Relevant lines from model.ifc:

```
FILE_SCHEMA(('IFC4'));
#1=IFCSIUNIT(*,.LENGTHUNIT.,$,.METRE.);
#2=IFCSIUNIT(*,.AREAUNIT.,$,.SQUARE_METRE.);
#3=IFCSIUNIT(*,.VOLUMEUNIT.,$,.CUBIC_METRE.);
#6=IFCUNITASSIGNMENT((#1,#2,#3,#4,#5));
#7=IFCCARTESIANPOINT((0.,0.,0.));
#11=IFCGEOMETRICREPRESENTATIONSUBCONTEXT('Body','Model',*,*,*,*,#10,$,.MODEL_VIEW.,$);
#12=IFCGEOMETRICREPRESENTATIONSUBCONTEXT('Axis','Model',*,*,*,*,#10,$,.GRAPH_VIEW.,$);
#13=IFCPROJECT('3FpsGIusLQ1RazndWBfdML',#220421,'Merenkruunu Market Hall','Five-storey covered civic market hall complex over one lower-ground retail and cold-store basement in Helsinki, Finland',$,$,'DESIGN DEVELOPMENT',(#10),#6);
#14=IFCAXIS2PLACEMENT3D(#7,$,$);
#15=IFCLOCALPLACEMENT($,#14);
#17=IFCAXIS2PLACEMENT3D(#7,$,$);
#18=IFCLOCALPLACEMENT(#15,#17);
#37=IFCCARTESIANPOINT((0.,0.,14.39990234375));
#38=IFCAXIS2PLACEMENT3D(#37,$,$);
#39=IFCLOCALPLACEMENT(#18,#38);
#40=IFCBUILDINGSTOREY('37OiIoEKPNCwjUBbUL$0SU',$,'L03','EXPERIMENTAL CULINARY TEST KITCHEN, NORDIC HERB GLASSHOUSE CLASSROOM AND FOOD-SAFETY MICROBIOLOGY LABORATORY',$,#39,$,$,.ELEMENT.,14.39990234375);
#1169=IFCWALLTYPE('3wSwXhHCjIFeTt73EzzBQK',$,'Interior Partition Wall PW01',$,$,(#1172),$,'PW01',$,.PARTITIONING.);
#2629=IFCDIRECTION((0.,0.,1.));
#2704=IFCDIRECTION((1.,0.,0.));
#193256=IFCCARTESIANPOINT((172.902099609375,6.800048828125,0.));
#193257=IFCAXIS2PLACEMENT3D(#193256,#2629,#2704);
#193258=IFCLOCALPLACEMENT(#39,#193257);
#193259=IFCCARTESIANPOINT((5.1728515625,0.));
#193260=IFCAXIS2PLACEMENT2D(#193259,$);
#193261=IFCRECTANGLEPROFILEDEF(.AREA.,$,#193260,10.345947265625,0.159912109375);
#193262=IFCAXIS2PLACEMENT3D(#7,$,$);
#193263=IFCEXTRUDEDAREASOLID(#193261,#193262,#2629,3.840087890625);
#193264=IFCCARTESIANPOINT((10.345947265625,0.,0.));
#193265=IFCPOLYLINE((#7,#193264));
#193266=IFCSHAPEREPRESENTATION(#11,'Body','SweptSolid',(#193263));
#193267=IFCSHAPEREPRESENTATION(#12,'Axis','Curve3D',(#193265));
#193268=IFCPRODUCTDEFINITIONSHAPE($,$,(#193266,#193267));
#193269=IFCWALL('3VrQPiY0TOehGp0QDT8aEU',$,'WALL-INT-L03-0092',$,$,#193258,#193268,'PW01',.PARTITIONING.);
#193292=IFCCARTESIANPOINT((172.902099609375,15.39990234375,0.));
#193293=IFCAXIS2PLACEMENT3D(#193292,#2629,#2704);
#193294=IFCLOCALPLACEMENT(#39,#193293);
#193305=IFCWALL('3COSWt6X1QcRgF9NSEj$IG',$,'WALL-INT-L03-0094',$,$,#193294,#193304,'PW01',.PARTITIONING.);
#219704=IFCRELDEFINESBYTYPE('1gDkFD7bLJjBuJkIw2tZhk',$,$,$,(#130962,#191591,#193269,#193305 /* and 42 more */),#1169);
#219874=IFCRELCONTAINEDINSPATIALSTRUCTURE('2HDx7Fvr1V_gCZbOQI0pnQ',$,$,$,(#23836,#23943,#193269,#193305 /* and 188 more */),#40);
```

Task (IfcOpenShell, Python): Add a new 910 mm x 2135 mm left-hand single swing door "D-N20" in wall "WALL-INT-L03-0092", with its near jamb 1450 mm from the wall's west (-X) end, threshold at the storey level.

```python
import numpy as np
import ifcopenshell
import ifcopenshell.api.feature
import ifcopenshell.api.geometry
import ifcopenshell.api.root
import ifcopenshell.api.spatial
import ifcopenshell.geom
import ifcopenshell.util.element
import ifcopenshell.util.placement
import ifcopenshell.util.representation
import ifcopenshell.util.shape
import ifcopenshell.util.unit

model = ifcopenshell.open("model.ifc")
unit_scale = ifcopenshell.util.unit.calculate_unit_scale(model)
settings = ifcopenshell.geom.settings()


def volume(element):
    """Net volume in cubic metres, openings subtracted."""
    shape = ifcopenshell.geom.create_shape(settings, element)
    return ifcopenshell.util.shape.get_volume(shape.geometry)


wall = model.by_id(193269)
storey = ifcopenshell.util.element.get_container(wall, ifc_class="IfcBuildingStorey")
context = ifcopenshell.util.representation.get_context(model, "Model", "Body", "MODEL_VIEW")
before = volume(wall)

width, height, from_end, sill = 0.91, 2.135, 1.45, 0.0  # metres

# The wall runs along its own X axis, and the end named is its -X end.
wall_shape = ifcopenshell.geom.create_shape(settings, wall)
x, y, z = ifcopenshell.util.shape.get_vertices(wall_shape.geometry).T
start = x.min() + from_end
face, thickness = float(y.min()), float(y.max() - y.min())
wall_matrix = ifcopenshell.util.placement.get_local_placement(wall.ObjectPlacement)
level = ifcopenshell.util.placement.get_local_placement(storey.ObjectPlacement)[2, 3]


def in_wall(x, y):
    """Placement at x, y metres in the wall's axes, at sill height."""
    matrix = wall_matrix.copy()
    matrix[:, 3] = wall_matrix @ np.array([x / unit_scale, y / unit_scale, 0.0, 1.0])
    matrix[2, 3] = level + sill / unit_scale
    return matrix


# Opening: a box that overshoots both wall faces by 50 mm.
opening = ifcopenshell.api.root.create_entity(model, ifc_class="IfcOpeningElement", predefined_type="OPENING")
box = ifcopenshell.api.geometry.add_wall_representation(
    model, context=context, length=width, height=height, thickness=thickness + 0.1
)
ifcopenshell.api.geometry.assign_representation(model, product=opening, representation=box)
ifcopenshell.api.geometry.edit_object_placement(model, product=opening, matrix=in_wall(start, face - 0.05), is_si=False)
ifcopenshell.api.feature.add_feature(model, feature=opening, element=wall)

door = ifcopenshell.api.root.create_entity(model, ifc_class="IfcDoor", name="D-N20", predefined_type="DOOR")
door.OverallWidth, door.OverallHeight = width / unit_scale, height / unit_scale
door.OperationType = "SINGLE_SWING_LEFT"
body = ifcopenshell.api.geometry.add_door_representation(
    model,
    context=context,
    overall_width=door.OverallWidth,
    overall_height=door.OverallHeight,
    operation_type="SINGLE_SWING_LEFT",
    lining_properties={"LiningDepth": thickness / unit_scale, "ThresholdDepth": thickness / unit_scale},
)
ifcopenshell.api.geometry.assign_representation(model, product=door, representation=body)
ifcopenshell.api.spatial.assign_container(model, products=[door], relating_structure=storey)
ifcopenshell.api.feature.add_filling(model, opening=opening, element=door)

# The lining spans the wall, so the door starts at the wall face.
ifcopenshell.api.geometry.edit_object_placement(model, product=door, matrix=in_wall(start, face), is_si=False)

after = volume(wall)

print(f"wall volume {before:.3f} -> {after:.3f} m3")

model.write("model_updated.ifc")
```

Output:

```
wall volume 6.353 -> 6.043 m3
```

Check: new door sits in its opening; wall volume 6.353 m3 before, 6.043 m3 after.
